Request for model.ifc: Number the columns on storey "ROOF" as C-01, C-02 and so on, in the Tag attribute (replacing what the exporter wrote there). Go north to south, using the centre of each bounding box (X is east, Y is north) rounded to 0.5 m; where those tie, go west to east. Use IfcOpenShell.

First a look at what the model holds.

```python
import ifcopenshell
import ifcopenshell.util.element
import ifcopenshell.util.placement

model = ifcopenshell.open("model.ifc")
print(model.schema)
storey = next(s for s in model.by_type("IfcBuildingStorey") if s.Name == "ROOF")
columns = [e for e in ifcopenshell.util.element.get_decomposition(storey) if e.is_a("IfcColumn")]
for e in sorted(columns, key=lambda e: e.id()):
    origin = ifcopenshell.util.placement.get_local_placement(e.ObjectPlacement)[:3, 3]
    print(e.id(), e.Tag, e.Name, origin.round(2) + 0.0, sep=" | ")
```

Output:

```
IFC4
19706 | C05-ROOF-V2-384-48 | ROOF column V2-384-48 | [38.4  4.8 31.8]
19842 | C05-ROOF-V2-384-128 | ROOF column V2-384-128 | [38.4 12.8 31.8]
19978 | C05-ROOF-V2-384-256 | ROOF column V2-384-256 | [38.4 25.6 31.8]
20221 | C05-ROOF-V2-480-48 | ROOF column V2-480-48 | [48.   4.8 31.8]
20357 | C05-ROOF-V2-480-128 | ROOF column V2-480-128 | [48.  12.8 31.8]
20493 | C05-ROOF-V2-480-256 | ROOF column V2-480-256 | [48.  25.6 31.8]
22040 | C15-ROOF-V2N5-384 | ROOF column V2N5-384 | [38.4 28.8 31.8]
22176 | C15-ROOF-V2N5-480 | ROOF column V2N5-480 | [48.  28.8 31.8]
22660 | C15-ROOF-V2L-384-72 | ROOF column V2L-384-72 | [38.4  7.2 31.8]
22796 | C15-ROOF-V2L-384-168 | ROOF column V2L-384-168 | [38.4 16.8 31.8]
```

```python
import ifcopenshell
import ifcopenshell.geom
import ifcopenshell.util.element
import ifcopenshell.util.shape

model = ifcopenshell.open("model.ifc")
settings = ifcopenshell.geom.settings()
settings.set("use-world-coords", True)


def centre(element):
    shape = ifcopenshell.geom.create_shape(settings, element)
    return ifcopenshell.util.shape.get_bbox_centroid(shape.geometry)


storey = next(s for s in model.by_type("IfcBuildingStorey") if s.Name == "ROOF")
columns = [e for e in ifcopenshell.util.element.get_decomposition(storey) if e.is_a("IfcColumn")]

# Insertion points can sit at a corner or the storey origin, so sort by the geometry (in metres).
centres = {e: centre(e) for e in columns}
columns.sort(key=lambda e: (-round(centres[e][1] / 0.5), centres[e][0]))

for i, e in enumerate(columns, start=1):
    number = f"C-{i:02d}"
    e.Tag = number
    print(e.id(), number)

model.write("model_rev.ifc")
```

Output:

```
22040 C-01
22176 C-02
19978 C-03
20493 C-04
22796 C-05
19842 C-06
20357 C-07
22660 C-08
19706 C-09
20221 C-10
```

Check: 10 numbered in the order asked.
